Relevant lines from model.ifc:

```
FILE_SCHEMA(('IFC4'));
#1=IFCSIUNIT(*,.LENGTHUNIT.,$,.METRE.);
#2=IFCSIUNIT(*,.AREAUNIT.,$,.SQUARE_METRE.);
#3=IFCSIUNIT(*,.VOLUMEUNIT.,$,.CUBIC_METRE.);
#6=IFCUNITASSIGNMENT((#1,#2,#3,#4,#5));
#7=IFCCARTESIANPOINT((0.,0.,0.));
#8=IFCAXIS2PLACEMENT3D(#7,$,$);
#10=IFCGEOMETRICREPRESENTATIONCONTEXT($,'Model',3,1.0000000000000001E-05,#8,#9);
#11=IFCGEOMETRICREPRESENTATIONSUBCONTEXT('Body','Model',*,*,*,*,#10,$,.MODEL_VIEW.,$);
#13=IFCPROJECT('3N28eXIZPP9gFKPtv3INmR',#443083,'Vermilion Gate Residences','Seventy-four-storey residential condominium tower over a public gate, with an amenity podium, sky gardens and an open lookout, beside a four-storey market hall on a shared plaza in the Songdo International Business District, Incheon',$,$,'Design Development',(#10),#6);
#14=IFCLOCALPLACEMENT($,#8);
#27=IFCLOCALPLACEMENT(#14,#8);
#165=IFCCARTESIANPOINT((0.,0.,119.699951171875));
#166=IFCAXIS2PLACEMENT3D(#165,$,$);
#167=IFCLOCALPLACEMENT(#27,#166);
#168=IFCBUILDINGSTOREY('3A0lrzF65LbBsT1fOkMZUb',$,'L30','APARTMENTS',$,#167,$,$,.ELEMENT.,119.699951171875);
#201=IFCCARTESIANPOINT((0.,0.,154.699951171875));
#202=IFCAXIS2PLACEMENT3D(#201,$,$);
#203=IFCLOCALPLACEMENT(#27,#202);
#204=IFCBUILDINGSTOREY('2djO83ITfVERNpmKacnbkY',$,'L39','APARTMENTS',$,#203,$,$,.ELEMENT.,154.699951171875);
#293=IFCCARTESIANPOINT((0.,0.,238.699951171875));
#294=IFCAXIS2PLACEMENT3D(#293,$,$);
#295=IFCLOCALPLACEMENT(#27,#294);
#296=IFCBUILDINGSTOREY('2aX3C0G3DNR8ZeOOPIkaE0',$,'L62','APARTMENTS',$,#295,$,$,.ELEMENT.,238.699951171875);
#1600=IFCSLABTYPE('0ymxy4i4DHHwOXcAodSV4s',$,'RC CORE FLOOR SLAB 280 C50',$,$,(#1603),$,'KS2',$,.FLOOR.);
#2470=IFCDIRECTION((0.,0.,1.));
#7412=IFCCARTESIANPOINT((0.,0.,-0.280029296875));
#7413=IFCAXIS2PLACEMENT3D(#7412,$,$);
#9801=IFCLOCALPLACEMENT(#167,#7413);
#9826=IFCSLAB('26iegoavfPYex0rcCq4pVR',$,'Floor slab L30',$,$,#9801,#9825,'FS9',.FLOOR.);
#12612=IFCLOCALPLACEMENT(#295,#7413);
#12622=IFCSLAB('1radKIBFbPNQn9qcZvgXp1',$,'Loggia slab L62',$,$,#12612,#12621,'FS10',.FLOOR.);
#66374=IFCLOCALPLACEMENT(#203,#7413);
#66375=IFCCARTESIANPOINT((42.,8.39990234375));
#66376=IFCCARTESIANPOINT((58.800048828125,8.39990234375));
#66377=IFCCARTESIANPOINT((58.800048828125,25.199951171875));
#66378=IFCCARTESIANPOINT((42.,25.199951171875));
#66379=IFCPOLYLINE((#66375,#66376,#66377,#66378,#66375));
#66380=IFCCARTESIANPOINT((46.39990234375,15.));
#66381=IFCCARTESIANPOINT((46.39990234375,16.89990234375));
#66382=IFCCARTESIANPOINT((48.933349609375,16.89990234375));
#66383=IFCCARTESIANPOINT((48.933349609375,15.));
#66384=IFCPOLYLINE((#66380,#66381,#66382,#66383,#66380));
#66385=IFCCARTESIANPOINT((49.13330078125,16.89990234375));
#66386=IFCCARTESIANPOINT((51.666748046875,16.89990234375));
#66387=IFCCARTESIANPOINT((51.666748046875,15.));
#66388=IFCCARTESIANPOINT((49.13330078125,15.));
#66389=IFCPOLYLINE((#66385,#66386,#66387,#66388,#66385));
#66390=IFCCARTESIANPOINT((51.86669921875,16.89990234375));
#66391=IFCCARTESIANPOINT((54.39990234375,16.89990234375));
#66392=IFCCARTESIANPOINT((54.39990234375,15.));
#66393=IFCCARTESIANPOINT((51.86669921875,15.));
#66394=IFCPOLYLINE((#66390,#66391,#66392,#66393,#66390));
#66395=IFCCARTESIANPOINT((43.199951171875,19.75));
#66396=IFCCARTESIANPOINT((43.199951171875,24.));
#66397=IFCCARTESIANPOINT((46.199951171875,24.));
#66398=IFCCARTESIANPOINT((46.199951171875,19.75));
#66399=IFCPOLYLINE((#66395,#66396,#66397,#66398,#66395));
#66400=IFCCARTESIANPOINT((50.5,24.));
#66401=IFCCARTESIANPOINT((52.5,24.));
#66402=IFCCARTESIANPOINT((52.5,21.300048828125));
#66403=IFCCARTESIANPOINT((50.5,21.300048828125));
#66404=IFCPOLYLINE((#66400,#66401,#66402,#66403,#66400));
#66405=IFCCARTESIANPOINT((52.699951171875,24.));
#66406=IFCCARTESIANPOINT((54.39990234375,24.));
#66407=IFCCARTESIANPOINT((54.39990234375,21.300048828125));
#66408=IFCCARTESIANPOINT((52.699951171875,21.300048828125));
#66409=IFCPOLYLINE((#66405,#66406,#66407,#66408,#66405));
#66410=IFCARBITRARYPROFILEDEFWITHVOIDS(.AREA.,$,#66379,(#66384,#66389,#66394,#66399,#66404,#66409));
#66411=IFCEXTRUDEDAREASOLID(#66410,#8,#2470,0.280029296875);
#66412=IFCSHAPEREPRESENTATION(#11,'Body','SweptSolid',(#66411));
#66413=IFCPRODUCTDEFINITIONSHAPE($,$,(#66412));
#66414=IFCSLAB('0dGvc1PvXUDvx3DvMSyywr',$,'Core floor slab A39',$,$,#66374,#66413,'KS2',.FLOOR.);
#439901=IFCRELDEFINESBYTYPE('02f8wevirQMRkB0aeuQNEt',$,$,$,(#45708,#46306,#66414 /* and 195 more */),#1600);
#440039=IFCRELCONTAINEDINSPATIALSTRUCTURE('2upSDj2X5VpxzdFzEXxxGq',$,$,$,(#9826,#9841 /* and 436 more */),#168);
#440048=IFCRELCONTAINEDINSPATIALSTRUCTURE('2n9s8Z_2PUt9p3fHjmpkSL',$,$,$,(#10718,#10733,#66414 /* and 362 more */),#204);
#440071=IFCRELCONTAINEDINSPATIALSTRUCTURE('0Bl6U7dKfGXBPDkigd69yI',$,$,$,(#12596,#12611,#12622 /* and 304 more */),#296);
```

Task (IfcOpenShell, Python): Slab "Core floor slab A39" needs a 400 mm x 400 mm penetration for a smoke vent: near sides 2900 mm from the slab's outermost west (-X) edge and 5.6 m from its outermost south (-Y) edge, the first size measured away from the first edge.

```python
import numpy as np
import ifcopenshell
import ifcopenshell.api.feature
import ifcopenshell.api.geometry
import ifcopenshell.api.root
import ifcopenshell.geom
import ifcopenshell.util.placement
import ifcopenshell.util.representation
import ifcopenshell.util.shape
import ifcopenshell.util.unit

model = ifcopenshell.open("model.ifc")
unit_scale = ifcopenshell.util.unit.calculate_unit_scale(model)
settings = ifcopenshell.geom.settings()


def volume(element):
    """Net volume in cubic metres, openings subtracted."""
    shape = ifcopenshell.geom.create_shape(settings, element)
    return ifcopenshell.util.shape.get_volume(shape.geometry)


slab = model.by_guid("0dGvc1PvXUDvx3DvMSyywr")
before = volume(slab)

# Extent in the slab's own axes, in metres. The edges named are its -X and -Y sides.
slab_shape = ifcopenshell.geom.create_shape(settings, slab)
vertices = ifcopenshell.util.shape.get_vertices(slab_shape.geometry)
x_min, y_min, bottom = vertices.min(axis=0)
top = vertices[:, 2].max()

opening = ifcopenshell.api.root.create_entity(model, ifc_class="IfcOpeningElement", name="Smoke vent opening", predefined_type="OPENING")
context = ifcopenshell.util.representation.get_context(model, "Model", "Body", "MODEL_VIEW")
width, depth = 0.4, 0.4
outline = [(0.0, 0.0), (width, 0.0), (width, depth), (0.0, depth), (0.0, 0.0)]
# Overshoot both faces by 50 mm so the cut is clean.
shape = ifcopenshell.api.geometry.add_slab_representation(
    model, context=context, depth=top - bottom + 0.1, polyline=outline
)
ifcopenshell.api.geometry.assign_representation(model, product=opening, representation=shape)

matrix = ifcopenshell.util.placement.get_local_placement(slab.ObjectPlacement)
matrix[:, 3] = matrix @ np.append(np.array([x_min + 2.9, y_min + 5.6, bottom - 0.05]) / unit_scale, 1.0)
ifcopenshell.api.geometry.edit_object_placement(model, product=opening, matrix=matrix, is_si=False)
ifcopenshell.api.feature.add_feature(model, feature=opening, element=slab)

after = volume(slab)

print(f"slab volume {before:.3f} -> {after:.3f} m3")

model.write("model_rev.ifc")
```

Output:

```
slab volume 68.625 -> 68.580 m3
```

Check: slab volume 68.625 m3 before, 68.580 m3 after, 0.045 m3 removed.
